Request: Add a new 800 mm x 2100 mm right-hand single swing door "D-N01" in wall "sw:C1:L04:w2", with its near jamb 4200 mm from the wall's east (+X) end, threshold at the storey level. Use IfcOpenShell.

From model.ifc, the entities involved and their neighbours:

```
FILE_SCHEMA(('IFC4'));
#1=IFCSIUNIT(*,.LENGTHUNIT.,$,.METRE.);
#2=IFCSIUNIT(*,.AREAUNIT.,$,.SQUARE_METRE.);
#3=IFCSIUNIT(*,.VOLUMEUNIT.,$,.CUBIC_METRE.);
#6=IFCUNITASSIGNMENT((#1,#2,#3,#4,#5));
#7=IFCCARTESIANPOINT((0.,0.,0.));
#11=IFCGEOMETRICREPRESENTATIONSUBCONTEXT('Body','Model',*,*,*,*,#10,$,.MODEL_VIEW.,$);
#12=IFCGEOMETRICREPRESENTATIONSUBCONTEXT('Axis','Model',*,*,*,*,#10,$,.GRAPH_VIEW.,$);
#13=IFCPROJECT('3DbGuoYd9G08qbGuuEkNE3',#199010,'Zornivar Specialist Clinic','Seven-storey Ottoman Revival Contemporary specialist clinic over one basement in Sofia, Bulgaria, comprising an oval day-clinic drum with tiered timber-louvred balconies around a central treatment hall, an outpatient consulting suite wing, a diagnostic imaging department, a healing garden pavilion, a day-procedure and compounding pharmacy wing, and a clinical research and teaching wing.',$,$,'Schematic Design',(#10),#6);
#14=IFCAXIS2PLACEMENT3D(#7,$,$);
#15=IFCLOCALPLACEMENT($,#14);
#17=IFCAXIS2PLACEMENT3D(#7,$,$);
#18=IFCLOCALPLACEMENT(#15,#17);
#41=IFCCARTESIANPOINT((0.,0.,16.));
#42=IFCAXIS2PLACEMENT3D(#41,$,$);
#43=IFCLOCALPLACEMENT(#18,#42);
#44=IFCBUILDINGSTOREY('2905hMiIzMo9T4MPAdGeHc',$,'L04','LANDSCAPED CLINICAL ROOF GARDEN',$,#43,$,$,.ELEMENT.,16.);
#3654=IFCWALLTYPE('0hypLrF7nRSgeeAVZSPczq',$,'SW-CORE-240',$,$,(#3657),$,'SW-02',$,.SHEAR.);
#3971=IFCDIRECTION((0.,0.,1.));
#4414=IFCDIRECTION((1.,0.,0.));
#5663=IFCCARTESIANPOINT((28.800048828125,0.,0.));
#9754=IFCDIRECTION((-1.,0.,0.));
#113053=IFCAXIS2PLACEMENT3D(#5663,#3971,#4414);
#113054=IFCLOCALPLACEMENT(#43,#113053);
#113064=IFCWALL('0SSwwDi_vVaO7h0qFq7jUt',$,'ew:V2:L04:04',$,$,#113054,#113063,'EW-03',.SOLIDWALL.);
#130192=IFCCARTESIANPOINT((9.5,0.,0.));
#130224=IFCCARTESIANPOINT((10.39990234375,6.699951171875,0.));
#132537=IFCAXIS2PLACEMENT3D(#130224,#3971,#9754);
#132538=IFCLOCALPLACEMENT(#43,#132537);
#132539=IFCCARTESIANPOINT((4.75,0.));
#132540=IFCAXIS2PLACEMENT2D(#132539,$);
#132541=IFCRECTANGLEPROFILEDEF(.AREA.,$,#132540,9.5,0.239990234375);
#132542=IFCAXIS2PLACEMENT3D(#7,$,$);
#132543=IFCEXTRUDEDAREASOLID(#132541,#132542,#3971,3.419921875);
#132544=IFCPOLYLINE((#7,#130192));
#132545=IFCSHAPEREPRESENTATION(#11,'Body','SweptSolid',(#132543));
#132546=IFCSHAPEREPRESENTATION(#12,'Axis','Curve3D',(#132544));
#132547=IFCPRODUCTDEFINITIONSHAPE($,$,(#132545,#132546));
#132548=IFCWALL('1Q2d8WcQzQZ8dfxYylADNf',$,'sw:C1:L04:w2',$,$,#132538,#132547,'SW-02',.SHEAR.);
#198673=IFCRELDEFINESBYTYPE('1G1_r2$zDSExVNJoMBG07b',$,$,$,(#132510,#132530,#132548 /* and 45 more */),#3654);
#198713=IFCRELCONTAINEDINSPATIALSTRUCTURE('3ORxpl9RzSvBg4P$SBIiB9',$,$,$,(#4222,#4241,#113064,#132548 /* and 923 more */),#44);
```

```python
import numpy as np
import ifcopenshell
import ifcopenshell.api.feature
import ifcopenshell.api.geometry
import ifcopenshell.api.root
import ifcopenshell.api.spatial
import ifcopenshell.geom
import ifcopenshell.util.element
import ifcopenshell.util.placement
import ifcopenshell.util.representation
import ifcopenshell.util.shape
import ifcopenshell.util.unit

model = ifcopenshell.open("model.ifc")
unit_scale = ifcopenshell.util.unit.calculate_unit_scale(model)
settings = ifcopenshell.geom.settings()


def volume(element):
    """Net volume in cubic metres, openings subtracted."""
    shape = ifcopenshell.geom.create_shape(settings, element)
    return ifcopenshell.util.shape.get_volume(shape.geometry)


wall = model.by_guid("1Q2d8WcQzQZ8dfxYylADNf")
storey = ifcopenshell.util.element.get_container(wall, ifc_class="IfcBuildingStorey")
context = ifcopenshell.util.representation.get_context(model, "Model", "Body", "MODEL_VIEW")
before = volume(wall)

width, height, from_end, sill = 0.8, 2.1, 4.2, 0.0  # metres

# The wall runs along its own X axis, and the end named is its -X end.
wall_shape = ifcopenshell.geom.create_shape(settings, wall)
x, y, z = ifcopenshell.util.shape.get_vertices(wall_shape.geometry).T
start = x.min() + from_end
face, thickness = float(y.min()), float(y.max() - y.min())
wall_matrix = ifcopenshell.util.placement.get_local_placement(wall.ObjectPlacement)
level = ifcopenshell.util.placement.get_local_placement(storey.ObjectPlacement)[2, 3]


def in_wall(x, y):
    """Placement at x, y metres in the wall's axes, at sill height."""
    matrix = wall_matrix.copy()
    matrix[:, 3] = wall_matrix @ np.array([x / unit_scale, y / unit_scale, 0.0, 1.0])
    matrix[2, 3] = level + sill / unit_scale
    return matrix


# Opening: a box that overshoots both wall faces by 50 mm.
opening = ifcopenshell.api.root.create_entity(model, ifc_class="IfcOpeningElement", predefined_type="OPENING")
box = ifcopenshell.api.geometry.add_wall_representation(
    model, context=context, length=width, height=height, thickness=thickness + 0.1
)
ifcopenshell.api.geometry.assign_representation(model, product=opening, representation=box)
ifcopenshell.api.geometry.edit_object_placement(model, product=opening, matrix=in_wall(start, face - 0.05), is_si=False)
ifcopenshell.api.feature.add_feature(model, feature=opening, element=wall)

door = ifcopenshell.api.root.create_entity(model, ifc_class="IfcDoor", name="D-N01", predefined_type="DOOR")
door.OverallWidth, door.OverallHeight = width / unit_scale, height / unit_scale
door.OperationType = "SINGLE_SWING_RIGHT"
body = ifcopenshell.api.geometry.add_door_representation(
    model,
    context=context,
    overall_width=door.OverallWidth,
    overall_height=door.OverallHeight,
    operation_type="SINGLE_SWING_RIGHT",
    lining_properties={"LiningDepth": thickness / unit_scale, "ThresholdDepth": thickness / unit_scale},
)
ifcopenshell.api.geometry.assign_representation(model, product=door, representation=body)
ifcopenshell.api.spatial.assign_container(model, products=[door], relating_structure=storey)
ifcopenshell.api.feature.add_filling(model, opening=opening, element=door)

# The lining spans the wall, so the door starts at the wall face.
ifcopenshell.api.geometry.edit_object_placement(model, product=door, matrix=in_wall(start, face), is_si=False)

after = volume(wall)

print(f"wall volume {before:.3f} -> {after:.3f} m3")

model.write("model_rev.ifc")
```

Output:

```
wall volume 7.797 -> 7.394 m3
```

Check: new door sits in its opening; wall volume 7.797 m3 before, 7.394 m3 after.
